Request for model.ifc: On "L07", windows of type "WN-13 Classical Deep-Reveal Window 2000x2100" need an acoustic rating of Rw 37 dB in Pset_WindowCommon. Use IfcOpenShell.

First a look at what the model holds.

```python
import ifcopenshell
import ifcopenshell.util.element

model = ifcopenshell.open("model.ifc")
print(model.schema)
storey = next(s for s in model.by_type("IfcBuildingStorey") if s.Name == "L07")
windows = [e for e in ifcopenshell.util.element.get_decomposition(storey) if e.is_a("IfcWindow")]
seen = {}
for e in windows:
    element_type = ifcopenshell.util.element.get_type(e)
    key = (element_type.Name if element_type != e and element_type else None, ifcopenshell.util.element.get_pset(e, "Pset_WindowCommon", "AcousticRating"))
    seen[key] = seen.get(key, 0) + 1
for (name, value), count in sorted(seen.items(), key=str):
    print(count, "x", name, "|", value)
```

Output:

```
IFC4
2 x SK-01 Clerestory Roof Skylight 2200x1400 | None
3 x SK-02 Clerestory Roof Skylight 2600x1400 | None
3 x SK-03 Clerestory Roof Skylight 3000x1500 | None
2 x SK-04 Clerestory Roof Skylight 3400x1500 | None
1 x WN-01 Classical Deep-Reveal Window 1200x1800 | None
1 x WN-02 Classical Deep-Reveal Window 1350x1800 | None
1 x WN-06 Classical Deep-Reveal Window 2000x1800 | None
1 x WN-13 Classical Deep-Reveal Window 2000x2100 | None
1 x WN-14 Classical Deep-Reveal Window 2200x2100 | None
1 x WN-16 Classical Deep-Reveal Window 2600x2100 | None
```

```python
import ifcopenshell
import ifcopenshell.api.pset
import ifcopenshell.util.element

model = ifcopenshell.open("model.ifc")

storey = next(s for s in model.by_type("IfcBuildingStorey") if s.Name == "L07")
windows = [e for e in ifcopenshell.util.element.get_decomposition(storey) if e.is_a("IfcWindow")]

count = 0
for e in windows:
    element_type = ifcopenshell.util.element.get_type(e)
    if element_type in (None, e) or element_type.Name != "WN-13 Classical Deep-Reveal Window 2000x2100":
        continue
    # add_pset returns the element's existing set when there is one.
    pset = ifcopenshell.api.pset.add_pset(model, product=e, name="Pset_WindowCommon")
    ifcopenshell.api.pset.edit_pset(model, pset=pset, properties={"AcousticRating": "Rw 37 dB"})
    count += 1

print(count, "windows updated")

model.write("model_updated.ifc")
```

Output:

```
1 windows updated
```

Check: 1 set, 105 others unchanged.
